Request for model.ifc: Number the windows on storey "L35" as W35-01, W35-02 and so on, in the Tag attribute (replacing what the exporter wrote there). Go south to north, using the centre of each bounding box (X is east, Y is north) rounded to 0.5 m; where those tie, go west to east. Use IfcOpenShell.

First a look at what the model holds.

```python
import ifcopenshell
import ifcopenshell.util.element
import ifcopenshell.util.placement

model = ifcopenshell.open("model.ifc")
print(model.schema)
storey = next(s for s in model.by_type("IfcBuildingStorey") if s.Name == "L35")
windows = [e for e in ifcopenshell.util.element.get_decomposition(storey) if e.is_a("IfcWindow")]
for e in sorted(windows, key=lambda e: e.id()):
    origin = ifcopenshell.util.placement.get_local_placement(e.ObjectPlacement)[:3, 3]
    print(e.id(), e.Tag, e.Name, origin.round(2) + 0.0, sep=" | ")
```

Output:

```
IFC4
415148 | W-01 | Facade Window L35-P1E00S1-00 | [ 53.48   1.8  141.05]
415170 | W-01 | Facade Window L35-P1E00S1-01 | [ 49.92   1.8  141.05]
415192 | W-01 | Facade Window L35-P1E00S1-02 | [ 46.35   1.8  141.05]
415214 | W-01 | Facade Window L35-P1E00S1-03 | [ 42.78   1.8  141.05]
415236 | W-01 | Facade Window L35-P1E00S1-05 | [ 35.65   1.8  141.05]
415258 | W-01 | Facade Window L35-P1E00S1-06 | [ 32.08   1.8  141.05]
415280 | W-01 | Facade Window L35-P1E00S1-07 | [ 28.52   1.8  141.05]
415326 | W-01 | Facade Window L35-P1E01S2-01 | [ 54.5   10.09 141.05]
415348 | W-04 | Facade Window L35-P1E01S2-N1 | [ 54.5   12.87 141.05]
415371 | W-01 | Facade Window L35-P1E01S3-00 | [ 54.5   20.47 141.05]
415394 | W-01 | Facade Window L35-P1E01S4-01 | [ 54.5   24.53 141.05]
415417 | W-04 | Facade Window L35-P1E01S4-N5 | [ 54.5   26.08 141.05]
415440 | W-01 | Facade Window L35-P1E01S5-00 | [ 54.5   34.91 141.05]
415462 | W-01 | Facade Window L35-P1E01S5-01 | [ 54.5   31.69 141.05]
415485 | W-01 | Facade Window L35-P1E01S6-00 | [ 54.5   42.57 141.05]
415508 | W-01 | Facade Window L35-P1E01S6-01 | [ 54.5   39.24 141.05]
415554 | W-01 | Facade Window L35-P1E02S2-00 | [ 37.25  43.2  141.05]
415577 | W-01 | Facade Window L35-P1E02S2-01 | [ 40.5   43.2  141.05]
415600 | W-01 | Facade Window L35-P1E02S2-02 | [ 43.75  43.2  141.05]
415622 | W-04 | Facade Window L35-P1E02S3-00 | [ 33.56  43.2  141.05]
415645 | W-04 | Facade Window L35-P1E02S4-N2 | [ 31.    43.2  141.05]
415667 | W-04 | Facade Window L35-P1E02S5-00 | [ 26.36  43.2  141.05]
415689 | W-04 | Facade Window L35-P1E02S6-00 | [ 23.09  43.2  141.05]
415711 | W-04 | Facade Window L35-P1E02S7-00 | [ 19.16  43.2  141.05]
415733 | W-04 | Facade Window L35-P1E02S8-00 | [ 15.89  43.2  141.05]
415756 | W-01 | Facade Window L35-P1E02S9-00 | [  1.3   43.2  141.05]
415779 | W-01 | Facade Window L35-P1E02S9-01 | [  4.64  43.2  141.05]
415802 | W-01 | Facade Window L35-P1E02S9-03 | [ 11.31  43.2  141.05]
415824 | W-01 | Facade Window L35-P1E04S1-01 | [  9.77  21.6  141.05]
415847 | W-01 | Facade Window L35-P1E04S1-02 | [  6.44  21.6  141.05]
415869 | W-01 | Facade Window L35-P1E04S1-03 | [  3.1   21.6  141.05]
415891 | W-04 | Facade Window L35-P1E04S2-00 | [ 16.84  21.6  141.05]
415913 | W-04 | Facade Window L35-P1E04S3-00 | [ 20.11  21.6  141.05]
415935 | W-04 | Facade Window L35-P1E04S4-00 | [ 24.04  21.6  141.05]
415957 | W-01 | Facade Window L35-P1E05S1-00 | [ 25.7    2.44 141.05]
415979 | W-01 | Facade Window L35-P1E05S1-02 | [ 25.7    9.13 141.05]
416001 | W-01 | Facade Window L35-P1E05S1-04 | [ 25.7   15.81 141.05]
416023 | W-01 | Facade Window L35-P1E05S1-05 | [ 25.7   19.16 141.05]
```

```python
import ifcopenshell
import ifcopenshell.geom
import ifcopenshell.util.element
import ifcopenshell.util.shape

model = ifcopenshell.open("model.ifc")
settings = ifcopenshell.geom.settings()
settings.set("use-world-coords", True)


def centre(element):
    shape = ifcopenshell.geom.create_shape(settings, element)
    return ifcopenshell.util.shape.get_bbox_centroid(shape.geometry)


storey = next(s for s in model.by_type("IfcBuildingStorey") if s.Name == "L35")
windows = [e for e in ifcopenshell.util.element.get_decomposition(storey) if e.is_a("IfcWindow")]

# Insertion points can sit at a corner or the storey origin, so sort by the geometry (in metres).
centres = {e: centre(e) for e in windows}
windows.sort(key=lambda e: (round(centres[e][1] / 0.5), centres[e][0]))

for i, e in enumerate(windows, start=1):
    number = f"W35-{i:02d}"
    e.Tag = number
    print(e.id(), number)

model.write("model_edited.ifc")
```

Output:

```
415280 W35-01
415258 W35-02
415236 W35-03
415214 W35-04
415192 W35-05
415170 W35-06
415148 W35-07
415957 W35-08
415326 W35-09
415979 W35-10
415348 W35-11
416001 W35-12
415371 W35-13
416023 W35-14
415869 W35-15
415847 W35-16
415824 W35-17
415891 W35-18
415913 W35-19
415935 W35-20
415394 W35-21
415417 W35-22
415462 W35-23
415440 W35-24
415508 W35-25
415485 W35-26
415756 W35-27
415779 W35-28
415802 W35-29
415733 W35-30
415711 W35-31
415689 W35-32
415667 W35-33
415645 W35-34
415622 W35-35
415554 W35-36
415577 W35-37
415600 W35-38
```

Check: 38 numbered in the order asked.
